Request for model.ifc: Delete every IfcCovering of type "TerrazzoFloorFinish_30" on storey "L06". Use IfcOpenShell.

First a look at what the model holds.

```python
import ifcopenshell
import ifcopenshell.util.element

model = ifcopenshell.open("model.ifc")
print(model.schema)
storey = next(s for s in model.by_type("IfcBuildingStorey") if s.Name == "L06")
coverings = [e for e in ifcopenshell.util.element.get_decomposition(storey) if e.is_a("IfcCovering")]
seen = {}
for e in coverings:
    element_type = ifcopenshell.util.element.get_type(e)
    name = element_type.Name if element_type not in (None, e) else None
    seen[name] = seen.get(name, 0) + 1
for name, count in sorted(seen.items(), key=str):
    print(count, "x", name)
```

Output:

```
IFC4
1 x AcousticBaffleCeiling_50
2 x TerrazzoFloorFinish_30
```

```python
import ifcopenshell
import ifcopenshell.api.root
import ifcopenshell.util.element

model = ifcopenshell.open("model.ifc")

storey = next(s for s in model.by_type("IfcBuildingStorey") if s.Name == "L06")
coverings = [e for e in ifcopenshell.util.element.get_decomposition(storey) if e.is_a("IfcCovering")]
targets = [e for e in coverings if (t := ifcopenshell.util.element.get_type(e)) not in (None, e) and t.Name == "TerrazzoFloorFinish_30"]

for e in targets:
    ifcopenshell.api.root.remove_product(model, product=e)
print(len(targets), "removed")

model.write("model_edited.ifc")
```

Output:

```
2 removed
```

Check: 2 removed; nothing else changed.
